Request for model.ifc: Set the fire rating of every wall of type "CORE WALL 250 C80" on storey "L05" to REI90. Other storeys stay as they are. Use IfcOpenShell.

First a look at what the model holds.

```python
import ifcopenshell
import ifcopenshell.util.element

model = ifcopenshell.open("model.ifc")
print(model.schema)
storey = next(s for s in model.by_type("IfcBuildingStorey") if s.Name == "L05")
walls = [e for e in ifcopenshell.util.element.get_decomposition(storey) if e.is_a("IfcWall")]
seen = {}
for e in walls:
    element_type = ifcopenshell.util.element.get_type(e)
    key = (element_type.Name if element_type != e and element_type else None, ifcopenshell.util.element.get_pset(e, "Pset_WallCommon", "FireRating"))
    seen[key] = seen.get(key, 0) + 1
for (name, value), count in sorted(seen.items(), key=str):
    print(count, "x", name, "|", value)
```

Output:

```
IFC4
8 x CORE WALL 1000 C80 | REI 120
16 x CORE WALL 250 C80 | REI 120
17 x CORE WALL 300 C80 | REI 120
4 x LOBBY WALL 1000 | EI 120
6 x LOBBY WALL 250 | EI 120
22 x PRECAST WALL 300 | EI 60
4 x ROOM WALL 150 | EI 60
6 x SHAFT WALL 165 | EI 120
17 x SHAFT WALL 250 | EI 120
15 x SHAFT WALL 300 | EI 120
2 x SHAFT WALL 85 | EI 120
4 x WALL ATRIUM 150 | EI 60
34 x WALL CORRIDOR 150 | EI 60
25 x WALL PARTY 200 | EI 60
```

```python
import ifcopenshell
import ifcopenshell.api.pset
import ifcopenshell.util.element

model = ifcopenshell.open("model.ifc")

storey = next(s for s in model.by_type("IfcBuildingStorey") if s.Name == "L05")
walls = [e for e in ifcopenshell.util.element.get_decomposition(storey) if e.is_a("IfcWall")]

count = 0
for e in walls:
    element_type = ifcopenshell.util.element.get_type(e)
    if element_type in (None, e) or element_type.Name != "CORE WALL 250 C80":
        continue
    found = ifcopenshell.util.element.get_pset(e, "Pset_WallCommon", should_inherit=False)
    if found:
        pset = model.by_id(found["id"])
        if len(ifcopenshell.util.element.get_elements_by_pset(pset)) > 1:
            pset = ifcopenshell.api.pset.unshare_pset(model, products=[e], pset=pset)[0]
    else:
        pset = ifcopenshell.api.pset.add_pset(model, product=e, name="Pset_WallCommon")
    ifcopenshell.api.pset.edit_pset(model, pset=pset, properties={"FireRating": "REI90"})
    count += 1

print(count, "walls updated")

model.write("model_v2.ifc")
```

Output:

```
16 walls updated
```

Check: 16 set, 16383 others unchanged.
